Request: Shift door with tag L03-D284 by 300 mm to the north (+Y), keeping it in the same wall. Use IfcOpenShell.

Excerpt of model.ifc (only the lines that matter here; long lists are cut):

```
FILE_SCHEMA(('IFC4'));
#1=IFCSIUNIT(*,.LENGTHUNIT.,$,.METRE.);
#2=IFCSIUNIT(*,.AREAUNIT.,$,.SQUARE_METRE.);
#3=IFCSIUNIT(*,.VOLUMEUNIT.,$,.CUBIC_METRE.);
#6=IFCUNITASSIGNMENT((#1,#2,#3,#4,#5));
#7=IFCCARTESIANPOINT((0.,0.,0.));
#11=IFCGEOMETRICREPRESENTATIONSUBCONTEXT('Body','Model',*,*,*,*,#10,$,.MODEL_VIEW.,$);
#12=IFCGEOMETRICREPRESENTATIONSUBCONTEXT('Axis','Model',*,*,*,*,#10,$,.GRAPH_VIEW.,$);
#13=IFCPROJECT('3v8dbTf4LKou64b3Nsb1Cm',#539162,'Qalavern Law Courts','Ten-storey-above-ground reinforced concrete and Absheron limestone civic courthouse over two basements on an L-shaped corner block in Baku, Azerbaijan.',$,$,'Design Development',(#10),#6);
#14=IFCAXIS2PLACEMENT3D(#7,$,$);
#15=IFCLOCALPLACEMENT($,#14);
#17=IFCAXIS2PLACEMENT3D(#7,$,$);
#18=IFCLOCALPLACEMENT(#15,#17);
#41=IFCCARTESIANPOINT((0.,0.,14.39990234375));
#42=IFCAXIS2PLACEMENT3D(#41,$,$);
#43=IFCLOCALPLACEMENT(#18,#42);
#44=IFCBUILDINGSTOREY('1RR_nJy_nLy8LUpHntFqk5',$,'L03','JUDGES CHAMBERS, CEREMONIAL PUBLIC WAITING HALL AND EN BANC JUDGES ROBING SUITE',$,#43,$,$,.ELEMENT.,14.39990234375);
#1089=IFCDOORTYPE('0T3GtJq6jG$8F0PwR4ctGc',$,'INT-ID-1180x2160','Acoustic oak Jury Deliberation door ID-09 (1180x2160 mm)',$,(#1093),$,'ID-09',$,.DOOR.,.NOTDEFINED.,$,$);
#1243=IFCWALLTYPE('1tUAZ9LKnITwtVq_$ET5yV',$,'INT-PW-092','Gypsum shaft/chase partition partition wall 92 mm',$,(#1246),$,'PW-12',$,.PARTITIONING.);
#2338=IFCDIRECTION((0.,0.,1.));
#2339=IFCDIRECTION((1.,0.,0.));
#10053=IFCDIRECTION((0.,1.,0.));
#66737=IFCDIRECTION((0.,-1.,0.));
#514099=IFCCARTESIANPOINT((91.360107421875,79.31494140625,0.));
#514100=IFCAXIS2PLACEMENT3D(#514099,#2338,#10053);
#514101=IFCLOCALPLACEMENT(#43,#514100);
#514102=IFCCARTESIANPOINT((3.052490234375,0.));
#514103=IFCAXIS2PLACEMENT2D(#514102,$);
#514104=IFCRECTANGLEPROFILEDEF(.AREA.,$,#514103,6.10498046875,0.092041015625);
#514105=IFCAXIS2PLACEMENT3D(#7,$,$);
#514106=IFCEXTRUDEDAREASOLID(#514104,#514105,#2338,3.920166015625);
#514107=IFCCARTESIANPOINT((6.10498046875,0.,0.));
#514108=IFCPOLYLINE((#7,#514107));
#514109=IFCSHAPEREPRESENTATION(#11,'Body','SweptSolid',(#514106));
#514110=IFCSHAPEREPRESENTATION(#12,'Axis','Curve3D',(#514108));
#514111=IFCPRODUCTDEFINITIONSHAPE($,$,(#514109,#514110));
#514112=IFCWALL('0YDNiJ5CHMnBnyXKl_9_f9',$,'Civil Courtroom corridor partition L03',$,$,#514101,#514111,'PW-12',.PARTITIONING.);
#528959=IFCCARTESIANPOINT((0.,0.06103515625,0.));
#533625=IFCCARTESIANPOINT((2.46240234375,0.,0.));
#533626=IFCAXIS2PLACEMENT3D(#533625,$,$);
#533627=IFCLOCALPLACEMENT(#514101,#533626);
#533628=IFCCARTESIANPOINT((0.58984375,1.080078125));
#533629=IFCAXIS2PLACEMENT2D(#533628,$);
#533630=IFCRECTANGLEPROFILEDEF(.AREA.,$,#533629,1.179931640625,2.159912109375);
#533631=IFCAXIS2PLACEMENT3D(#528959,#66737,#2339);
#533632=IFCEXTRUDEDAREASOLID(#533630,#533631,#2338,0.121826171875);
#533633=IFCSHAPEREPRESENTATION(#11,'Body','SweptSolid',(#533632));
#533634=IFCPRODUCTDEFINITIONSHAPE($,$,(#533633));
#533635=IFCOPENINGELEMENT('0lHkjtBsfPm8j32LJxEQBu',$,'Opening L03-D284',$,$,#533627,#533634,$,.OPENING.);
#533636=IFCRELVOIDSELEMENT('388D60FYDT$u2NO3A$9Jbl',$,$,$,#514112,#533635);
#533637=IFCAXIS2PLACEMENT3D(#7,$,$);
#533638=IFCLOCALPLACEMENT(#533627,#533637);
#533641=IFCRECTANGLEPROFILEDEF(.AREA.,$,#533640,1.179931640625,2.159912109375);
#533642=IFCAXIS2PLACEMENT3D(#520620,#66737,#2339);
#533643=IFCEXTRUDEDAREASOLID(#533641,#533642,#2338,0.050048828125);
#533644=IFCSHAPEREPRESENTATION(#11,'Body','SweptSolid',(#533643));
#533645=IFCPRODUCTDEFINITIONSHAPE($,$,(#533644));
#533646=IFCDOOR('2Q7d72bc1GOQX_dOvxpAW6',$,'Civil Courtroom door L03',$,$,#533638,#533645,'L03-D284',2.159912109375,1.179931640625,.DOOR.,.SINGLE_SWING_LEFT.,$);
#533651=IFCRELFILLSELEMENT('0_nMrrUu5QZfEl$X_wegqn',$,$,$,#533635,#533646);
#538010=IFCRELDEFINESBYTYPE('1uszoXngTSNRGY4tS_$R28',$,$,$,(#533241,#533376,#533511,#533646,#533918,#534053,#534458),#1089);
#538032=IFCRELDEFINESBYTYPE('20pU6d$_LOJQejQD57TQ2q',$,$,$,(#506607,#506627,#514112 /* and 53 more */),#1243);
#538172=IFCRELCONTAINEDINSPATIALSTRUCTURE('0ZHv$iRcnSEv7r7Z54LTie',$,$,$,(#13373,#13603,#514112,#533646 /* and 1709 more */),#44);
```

```python
import ifcopenshell
import ifcopenshell.api.geometry
import ifcopenshell.util.placement

model = ifcopenshell.open("model.ifc")

door = model.by_guid("2Q7d72bc1GOQX_dOvxpAW6")
opening = door.FillsVoids[0].RelatingOpeningElement
wall = opening.VoidsElements[0].RelatingBuildingElement

wall_matrix = ifcopenshell.util.placement.get_local_placement(wall.ObjectPlacement)
shift = wall_matrix[:3, 0] * 0.3
before = ifcopenshell.util.placement.get_local_placement(door.ObjectPlacement)[:3, 3].copy()

# The door is placed relative to its opening, so it follows when the opening moves.
matrix = ifcopenshell.util.placement.get_local_placement(opening.ObjectPlacement)
matrix[:3, 3] += shift
ifcopenshell.api.geometry.edit_object_placement(
    model, product=opening, matrix=matrix, is_si=False, should_transform_children=True
)

after = ifcopenshell.util.placement.get_local_placement(door.ObjectPlacement)[:3, 3]
print("door moved by", (after - before).round(3) + 0.0)

model.write("model_updated.ifc")
```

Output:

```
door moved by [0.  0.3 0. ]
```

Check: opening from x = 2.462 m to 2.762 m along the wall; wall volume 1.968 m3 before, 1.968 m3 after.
